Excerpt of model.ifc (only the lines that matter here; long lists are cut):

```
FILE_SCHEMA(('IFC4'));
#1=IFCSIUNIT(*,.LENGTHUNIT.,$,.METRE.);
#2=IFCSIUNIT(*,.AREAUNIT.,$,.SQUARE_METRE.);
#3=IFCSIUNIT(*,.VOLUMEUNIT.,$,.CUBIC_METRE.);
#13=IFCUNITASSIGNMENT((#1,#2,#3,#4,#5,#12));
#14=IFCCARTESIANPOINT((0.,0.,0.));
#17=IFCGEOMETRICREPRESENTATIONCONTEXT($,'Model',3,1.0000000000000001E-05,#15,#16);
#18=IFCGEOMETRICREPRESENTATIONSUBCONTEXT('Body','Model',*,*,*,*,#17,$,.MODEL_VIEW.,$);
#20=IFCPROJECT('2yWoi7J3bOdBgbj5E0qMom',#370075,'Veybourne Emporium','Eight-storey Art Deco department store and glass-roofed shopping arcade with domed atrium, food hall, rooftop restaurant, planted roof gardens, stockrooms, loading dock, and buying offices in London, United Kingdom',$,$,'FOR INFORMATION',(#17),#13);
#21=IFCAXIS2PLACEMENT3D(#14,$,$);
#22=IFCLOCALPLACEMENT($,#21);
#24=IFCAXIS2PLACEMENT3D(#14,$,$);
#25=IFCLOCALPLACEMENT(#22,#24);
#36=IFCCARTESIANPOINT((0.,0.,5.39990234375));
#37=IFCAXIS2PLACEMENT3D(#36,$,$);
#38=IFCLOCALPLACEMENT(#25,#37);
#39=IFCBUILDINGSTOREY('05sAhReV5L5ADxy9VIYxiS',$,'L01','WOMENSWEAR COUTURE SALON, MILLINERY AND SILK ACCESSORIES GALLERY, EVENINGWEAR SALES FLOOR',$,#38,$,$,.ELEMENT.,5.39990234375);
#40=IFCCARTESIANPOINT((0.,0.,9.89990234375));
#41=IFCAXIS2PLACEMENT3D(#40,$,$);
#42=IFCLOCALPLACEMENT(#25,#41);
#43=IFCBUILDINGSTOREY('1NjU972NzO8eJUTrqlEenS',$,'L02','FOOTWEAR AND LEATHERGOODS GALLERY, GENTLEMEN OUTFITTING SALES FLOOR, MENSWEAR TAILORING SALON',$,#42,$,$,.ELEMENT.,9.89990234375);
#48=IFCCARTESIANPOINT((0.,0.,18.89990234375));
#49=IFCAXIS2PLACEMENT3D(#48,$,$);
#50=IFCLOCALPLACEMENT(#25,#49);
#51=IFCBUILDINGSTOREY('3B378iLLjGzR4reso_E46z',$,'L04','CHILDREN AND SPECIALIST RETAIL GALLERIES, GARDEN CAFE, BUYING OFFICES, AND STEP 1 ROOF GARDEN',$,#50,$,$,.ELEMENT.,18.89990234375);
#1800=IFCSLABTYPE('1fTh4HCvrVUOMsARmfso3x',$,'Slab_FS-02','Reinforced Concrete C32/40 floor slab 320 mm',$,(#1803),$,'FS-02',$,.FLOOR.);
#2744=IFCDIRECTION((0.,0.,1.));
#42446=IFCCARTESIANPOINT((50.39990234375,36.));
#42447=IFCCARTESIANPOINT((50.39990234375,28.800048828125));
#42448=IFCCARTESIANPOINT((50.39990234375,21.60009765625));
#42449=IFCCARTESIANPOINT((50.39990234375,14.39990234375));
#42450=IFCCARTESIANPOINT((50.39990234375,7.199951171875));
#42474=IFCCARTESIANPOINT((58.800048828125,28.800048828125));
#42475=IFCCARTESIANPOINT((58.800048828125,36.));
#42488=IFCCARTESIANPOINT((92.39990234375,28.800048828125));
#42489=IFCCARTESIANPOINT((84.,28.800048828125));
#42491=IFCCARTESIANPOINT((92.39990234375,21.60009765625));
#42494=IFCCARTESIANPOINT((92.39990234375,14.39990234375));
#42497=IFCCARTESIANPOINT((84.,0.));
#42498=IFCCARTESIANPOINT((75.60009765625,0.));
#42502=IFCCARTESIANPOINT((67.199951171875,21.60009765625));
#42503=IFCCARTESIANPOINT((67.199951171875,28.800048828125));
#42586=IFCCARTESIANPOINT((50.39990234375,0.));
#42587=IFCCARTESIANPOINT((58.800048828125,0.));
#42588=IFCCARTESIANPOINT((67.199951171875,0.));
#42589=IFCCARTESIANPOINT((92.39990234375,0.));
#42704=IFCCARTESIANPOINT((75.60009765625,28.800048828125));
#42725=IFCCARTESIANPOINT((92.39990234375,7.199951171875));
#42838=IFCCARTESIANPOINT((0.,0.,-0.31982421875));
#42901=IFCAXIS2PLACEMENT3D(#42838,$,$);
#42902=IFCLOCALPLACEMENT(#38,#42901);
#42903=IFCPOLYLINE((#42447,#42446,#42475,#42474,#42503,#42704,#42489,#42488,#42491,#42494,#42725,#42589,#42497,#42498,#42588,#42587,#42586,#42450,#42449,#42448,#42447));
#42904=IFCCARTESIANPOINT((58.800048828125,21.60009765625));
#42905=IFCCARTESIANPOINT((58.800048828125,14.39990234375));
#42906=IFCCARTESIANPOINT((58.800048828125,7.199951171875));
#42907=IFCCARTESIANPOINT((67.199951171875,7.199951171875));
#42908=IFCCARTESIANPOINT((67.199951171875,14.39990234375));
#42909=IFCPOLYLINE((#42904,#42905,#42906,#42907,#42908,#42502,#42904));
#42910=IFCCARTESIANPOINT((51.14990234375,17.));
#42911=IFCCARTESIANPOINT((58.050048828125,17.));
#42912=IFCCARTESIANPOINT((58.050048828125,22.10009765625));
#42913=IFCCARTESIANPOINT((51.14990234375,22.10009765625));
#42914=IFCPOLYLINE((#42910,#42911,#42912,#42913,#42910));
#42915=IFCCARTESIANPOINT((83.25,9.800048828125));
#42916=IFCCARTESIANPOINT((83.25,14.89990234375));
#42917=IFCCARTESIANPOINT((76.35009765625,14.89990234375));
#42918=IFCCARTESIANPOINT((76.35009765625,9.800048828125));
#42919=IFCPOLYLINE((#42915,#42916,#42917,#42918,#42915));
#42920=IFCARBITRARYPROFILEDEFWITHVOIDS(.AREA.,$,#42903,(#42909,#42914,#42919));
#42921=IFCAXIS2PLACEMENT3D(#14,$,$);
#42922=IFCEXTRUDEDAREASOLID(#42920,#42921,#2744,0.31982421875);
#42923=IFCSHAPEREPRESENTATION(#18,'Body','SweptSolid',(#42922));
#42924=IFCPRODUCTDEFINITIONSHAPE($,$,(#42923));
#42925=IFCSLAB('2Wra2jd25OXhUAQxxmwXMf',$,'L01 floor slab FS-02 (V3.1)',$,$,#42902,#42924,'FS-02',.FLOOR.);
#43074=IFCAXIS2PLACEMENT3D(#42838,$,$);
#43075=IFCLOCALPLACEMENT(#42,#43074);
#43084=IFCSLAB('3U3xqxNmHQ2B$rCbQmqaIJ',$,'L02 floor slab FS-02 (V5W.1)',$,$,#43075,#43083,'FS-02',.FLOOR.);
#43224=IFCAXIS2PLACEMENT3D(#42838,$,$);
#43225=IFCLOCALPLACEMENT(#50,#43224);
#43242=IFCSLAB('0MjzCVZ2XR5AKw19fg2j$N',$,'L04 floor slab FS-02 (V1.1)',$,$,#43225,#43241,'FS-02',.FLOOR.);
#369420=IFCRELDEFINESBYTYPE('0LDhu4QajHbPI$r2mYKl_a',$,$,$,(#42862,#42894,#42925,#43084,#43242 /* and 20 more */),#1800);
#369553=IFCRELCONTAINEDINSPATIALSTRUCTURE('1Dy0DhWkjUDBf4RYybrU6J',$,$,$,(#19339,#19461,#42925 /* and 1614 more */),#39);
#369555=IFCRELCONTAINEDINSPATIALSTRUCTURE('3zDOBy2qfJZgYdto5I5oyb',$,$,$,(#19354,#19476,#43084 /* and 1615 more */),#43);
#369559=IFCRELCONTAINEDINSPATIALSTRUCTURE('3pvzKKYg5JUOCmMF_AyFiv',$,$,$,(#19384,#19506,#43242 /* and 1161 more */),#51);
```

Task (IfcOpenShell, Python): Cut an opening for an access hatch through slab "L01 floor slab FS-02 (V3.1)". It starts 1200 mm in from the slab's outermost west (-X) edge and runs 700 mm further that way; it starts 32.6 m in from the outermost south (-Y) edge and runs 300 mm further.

```python
import numpy as np
import ifcopenshell
import ifcopenshell.api.feature
import ifcopenshell.api.geometry
import ifcopenshell.api.root
import ifcopenshell.geom
import ifcopenshell.util.placement
import ifcopenshell.util.representation
import ifcopenshell.util.shape
import ifcopenshell.util.unit

model = ifcopenshell.open("model.ifc")
unit_scale = ifcopenshell.util.unit.calculate_unit_scale(model)
settings = ifcopenshell.geom.settings()


def volume(element):
    """Net volume in cubic metres, openings subtracted."""
    shape = ifcopenshell.geom.create_shape(settings, element)
    return ifcopenshell.util.shape.get_volume(shape.geometry)


slab = model.by_guid("2Wra2jd25OXhUAQxxmwXMf")
before = volume(slab)

# Extent in the slab's own axes, in metres. The edges named are its -X and -Y sides.
slab_shape = ifcopenshell.geom.create_shape(settings, slab)
vertices = ifcopenshell.util.shape.get_vertices(slab_shape.geometry)
x_min, y_min, bottom = vertices.min(axis=0)
top = vertices[:, 2].max()

opening = ifcopenshell.api.root.create_entity(model, ifc_class="IfcOpeningElement", name="Access hatch opening", predefined_type="OPENING")
context = ifcopenshell.util.representation.get_context(model, "Model", "Body", "MODEL_VIEW")
width, depth = 0.7, 0.3
outline = [(0.0, 0.0), (width, 0.0), (width, depth), (0.0, depth), (0.0, 0.0)]
# Overshoot both faces by 50 mm so the cut is clean.
shape = ifcopenshell.api.geometry.add_slab_representation(
    model, context=context, depth=top - bottom + 0.1, polyline=outline
)
ifcopenshell.api.geometry.assign_representation(model, product=opening, representation=shape)

matrix = ifcopenshell.util.placement.get_local_placement(slab.ObjectPlacement)
matrix[:, 3] = matrix @ np.append(np.array([x_min + 1.2, y_min + 32.6, bottom - 0.05]) / unit_scale, 1.0)
ifcopenshell.api.geometry.edit_object_placement(model, product=opening, matrix=matrix, is_si=False)
ifcopenshell.api.feature.add_feature(model, feature=opening, element=slab)

after = volume(slab)

print(f"slab volume {before:.3f} -> {after:.3f} m3")

model.write("model_edited.ifc")
```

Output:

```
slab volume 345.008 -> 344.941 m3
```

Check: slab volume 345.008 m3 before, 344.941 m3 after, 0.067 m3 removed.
